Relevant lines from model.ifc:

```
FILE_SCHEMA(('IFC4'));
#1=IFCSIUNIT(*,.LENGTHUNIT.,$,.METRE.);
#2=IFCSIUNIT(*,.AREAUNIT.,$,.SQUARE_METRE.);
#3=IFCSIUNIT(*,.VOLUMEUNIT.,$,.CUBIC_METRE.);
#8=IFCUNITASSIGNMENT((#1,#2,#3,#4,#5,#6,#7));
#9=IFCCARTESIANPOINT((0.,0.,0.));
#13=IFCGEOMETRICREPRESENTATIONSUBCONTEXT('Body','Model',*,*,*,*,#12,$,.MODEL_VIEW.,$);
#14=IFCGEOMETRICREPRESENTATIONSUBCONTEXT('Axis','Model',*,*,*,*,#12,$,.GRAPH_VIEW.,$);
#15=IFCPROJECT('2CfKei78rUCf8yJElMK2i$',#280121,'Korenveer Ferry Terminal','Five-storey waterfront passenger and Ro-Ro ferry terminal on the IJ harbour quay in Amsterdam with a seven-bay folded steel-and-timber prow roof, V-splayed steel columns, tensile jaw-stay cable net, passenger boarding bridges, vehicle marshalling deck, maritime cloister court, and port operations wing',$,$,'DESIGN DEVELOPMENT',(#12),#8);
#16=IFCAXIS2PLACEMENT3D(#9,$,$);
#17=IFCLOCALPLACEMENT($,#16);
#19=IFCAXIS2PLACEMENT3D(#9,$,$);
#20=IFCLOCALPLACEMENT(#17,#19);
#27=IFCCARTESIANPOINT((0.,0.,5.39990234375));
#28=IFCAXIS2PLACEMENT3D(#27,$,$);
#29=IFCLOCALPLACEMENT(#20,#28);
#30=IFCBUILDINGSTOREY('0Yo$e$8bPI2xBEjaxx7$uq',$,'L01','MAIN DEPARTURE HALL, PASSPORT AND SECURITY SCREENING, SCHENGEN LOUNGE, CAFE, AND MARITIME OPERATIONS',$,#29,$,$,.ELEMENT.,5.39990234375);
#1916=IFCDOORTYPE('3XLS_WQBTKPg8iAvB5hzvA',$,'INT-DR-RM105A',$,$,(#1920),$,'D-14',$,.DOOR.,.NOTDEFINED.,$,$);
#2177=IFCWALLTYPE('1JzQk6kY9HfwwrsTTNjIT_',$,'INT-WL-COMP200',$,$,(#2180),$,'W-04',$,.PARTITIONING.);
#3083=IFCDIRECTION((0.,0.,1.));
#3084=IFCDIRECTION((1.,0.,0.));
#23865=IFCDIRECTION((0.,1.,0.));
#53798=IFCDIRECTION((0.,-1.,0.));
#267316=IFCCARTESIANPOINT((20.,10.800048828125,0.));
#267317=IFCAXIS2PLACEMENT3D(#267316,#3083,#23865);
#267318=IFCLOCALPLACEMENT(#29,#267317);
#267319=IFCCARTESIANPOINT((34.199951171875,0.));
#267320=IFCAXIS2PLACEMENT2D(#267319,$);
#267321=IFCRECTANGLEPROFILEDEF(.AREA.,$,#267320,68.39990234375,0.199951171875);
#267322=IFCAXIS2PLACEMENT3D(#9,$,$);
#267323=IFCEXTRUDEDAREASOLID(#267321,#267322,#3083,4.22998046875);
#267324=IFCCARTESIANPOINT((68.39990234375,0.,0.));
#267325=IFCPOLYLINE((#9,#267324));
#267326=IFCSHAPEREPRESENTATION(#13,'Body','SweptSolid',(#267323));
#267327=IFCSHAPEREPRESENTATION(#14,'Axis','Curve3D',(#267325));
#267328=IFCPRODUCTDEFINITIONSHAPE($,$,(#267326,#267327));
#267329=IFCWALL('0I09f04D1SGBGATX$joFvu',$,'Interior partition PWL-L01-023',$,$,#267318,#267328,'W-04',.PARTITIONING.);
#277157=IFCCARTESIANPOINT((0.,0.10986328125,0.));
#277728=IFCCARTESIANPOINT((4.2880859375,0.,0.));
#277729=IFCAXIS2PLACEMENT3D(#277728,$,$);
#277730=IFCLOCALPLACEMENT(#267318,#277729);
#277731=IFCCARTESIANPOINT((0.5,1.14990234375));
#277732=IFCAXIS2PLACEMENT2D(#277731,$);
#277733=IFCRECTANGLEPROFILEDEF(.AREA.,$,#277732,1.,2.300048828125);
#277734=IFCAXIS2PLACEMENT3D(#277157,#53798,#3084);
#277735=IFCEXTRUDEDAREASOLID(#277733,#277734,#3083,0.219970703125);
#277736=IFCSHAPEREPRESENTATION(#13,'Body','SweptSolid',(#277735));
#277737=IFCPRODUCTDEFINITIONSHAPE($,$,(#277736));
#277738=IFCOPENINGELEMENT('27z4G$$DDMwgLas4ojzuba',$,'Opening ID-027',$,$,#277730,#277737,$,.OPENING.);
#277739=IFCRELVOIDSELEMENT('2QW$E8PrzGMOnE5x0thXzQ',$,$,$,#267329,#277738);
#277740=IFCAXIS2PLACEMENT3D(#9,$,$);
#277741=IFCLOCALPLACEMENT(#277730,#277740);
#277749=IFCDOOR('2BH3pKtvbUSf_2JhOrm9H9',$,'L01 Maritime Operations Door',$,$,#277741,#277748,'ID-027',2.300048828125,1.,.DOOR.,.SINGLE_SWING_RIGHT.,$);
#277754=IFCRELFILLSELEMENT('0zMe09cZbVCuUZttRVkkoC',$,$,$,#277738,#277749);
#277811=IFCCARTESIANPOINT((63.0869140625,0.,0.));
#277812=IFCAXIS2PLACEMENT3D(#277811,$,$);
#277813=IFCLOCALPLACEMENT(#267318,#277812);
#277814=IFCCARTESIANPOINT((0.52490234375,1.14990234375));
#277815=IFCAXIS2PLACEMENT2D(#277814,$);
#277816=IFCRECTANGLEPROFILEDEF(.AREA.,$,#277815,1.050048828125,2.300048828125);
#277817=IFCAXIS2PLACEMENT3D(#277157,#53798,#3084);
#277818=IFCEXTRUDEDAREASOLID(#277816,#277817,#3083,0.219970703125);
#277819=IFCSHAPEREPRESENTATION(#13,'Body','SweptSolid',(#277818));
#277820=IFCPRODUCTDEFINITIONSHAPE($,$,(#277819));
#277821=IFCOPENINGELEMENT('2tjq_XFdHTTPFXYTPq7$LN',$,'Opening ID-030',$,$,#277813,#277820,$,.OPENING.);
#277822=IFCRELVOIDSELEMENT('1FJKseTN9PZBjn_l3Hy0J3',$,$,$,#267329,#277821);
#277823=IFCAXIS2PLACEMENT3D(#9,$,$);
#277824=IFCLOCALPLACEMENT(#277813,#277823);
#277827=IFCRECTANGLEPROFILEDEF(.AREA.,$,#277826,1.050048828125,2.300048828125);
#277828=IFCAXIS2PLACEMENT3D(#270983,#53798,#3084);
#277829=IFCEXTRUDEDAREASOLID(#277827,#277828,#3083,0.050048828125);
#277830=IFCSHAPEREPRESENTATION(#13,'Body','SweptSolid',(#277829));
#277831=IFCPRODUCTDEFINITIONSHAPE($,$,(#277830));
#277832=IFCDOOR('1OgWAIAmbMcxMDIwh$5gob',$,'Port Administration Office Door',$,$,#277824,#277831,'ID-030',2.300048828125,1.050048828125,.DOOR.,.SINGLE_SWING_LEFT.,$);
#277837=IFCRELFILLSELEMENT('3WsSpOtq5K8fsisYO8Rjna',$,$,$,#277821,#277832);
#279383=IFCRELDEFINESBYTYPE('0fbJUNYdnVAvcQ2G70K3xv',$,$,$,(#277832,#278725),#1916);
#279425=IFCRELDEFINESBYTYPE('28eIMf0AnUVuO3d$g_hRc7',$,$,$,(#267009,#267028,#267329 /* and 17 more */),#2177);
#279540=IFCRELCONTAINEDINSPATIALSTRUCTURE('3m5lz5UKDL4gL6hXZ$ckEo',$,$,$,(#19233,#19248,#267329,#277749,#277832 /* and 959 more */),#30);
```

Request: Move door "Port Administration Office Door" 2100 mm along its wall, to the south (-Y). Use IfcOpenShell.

```python
import ifcopenshell
import ifcopenshell.api.geometry
import ifcopenshell.util.placement
import ifcopenshell.util.unit

model = ifcopenshell.open("model.ifc")
unit_scale = ifcopenshell.util.unit.calculate_unit_scale(model)

door = model.by_guid("1OgWAIAmbMcxMDIwh$5gob")
opening = door.FillsVoids[0].RelatingOpeningElement
wall = opening.VoidsElements[0].RelatingBuildingElement

wall_matrix = ifcopenshell.util.placement.get_local_placement(wall.ObjectPlacement)
shift = wall_matrix[:3, 0] * -2.1 / unit_scale
before = ifcopenshell.util.placement.get_local_placement(door.ObjectPlacement)[:3, 3].copy()

# The door is placed relative to its opening, so it follows when the opening moves.
matrix = ifcopenshell.util.placement.get_local_placement(opening.ObjectPlacement)
matrix[:3, 3] += shift
ifcopenshell.api.geometry.edit_object_placement(
    model, product=opening, matrix=matrix, is_si=False, should_transform_children=True
)

after = ifcopenshell.util.placement.get_local_placement(door.ObjectPlacement)[:3, 3]
print("door moved by", (after - before).round(3) + 0.0)

model.write("model-out.ifc")
```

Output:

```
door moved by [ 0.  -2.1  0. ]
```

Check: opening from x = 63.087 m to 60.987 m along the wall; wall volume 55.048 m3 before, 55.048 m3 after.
